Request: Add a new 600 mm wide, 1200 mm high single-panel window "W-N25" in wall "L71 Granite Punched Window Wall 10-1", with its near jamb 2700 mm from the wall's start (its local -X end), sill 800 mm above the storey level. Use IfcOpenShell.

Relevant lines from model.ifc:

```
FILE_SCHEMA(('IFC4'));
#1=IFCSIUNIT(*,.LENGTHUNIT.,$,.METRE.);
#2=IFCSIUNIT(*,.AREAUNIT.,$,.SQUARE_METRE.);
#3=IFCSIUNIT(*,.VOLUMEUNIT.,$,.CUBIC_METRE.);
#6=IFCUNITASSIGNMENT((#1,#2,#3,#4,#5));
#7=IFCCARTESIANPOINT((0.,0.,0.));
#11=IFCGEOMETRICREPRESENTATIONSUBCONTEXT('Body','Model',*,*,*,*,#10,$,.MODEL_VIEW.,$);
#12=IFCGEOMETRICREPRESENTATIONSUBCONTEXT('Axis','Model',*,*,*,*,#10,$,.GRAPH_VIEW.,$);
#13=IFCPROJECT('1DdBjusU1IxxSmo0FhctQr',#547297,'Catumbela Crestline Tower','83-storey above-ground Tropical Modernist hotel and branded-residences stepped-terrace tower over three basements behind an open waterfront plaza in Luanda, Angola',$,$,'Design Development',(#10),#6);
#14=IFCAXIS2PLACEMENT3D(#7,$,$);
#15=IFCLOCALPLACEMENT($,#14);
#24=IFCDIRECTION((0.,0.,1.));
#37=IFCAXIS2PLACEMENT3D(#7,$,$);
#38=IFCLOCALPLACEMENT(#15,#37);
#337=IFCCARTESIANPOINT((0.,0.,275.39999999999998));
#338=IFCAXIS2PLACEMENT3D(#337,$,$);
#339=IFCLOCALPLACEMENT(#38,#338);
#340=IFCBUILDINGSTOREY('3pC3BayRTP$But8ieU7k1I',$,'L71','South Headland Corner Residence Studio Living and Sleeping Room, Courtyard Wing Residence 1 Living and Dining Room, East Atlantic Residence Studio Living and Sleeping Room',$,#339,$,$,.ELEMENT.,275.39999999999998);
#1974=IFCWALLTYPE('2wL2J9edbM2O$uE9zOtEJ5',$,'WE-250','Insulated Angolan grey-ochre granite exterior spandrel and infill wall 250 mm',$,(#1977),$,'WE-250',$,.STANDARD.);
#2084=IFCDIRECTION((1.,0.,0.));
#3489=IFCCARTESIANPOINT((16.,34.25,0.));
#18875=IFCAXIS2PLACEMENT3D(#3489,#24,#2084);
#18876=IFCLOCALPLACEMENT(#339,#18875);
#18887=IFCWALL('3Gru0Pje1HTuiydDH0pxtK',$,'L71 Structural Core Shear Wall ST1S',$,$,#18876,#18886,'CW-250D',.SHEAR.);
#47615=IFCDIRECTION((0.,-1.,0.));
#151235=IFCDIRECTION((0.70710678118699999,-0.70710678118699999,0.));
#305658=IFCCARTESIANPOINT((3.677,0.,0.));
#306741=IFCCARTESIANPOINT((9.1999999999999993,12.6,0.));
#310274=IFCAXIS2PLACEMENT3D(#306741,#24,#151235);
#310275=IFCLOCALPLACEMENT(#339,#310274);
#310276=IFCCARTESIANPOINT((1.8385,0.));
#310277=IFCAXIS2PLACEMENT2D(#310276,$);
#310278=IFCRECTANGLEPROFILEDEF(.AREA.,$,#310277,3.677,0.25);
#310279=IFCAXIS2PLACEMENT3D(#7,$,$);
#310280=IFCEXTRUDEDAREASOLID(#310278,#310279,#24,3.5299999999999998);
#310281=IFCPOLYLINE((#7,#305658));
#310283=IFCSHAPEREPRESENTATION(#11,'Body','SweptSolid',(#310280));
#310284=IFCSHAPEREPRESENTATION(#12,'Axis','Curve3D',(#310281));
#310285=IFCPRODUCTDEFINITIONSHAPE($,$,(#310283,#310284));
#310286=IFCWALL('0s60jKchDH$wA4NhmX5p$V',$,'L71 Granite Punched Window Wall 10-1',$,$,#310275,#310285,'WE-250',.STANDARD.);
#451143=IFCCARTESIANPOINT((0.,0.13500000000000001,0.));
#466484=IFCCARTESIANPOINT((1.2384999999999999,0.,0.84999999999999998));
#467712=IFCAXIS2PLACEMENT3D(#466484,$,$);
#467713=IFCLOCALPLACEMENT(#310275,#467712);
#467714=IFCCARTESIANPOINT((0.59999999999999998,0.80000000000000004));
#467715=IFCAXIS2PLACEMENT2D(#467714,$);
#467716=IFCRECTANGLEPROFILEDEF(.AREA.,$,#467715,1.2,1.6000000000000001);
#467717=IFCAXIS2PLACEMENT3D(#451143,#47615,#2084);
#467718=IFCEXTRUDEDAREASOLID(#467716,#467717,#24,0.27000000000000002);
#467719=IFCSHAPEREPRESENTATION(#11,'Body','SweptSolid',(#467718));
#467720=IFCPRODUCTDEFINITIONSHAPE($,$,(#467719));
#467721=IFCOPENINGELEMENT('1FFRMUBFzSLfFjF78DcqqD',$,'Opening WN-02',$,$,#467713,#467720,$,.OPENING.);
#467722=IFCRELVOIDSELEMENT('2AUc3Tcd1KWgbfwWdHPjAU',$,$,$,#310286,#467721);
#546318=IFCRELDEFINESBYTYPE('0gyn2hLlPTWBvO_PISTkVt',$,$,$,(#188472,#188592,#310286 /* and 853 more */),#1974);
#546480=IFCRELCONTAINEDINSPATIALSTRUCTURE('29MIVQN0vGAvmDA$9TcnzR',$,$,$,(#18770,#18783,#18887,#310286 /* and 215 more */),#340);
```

```python
import numpy as np
import ifcopenshell
import ifcopenshell.api.feature
import ifcopenshell.api.geometry
import ifcopenshell.api.root
import ifcopenshell.api.spatial
import ifcopenshell.geom
import ifcopenshell.util.element
import ifcopenshell.util.placement
import ifcopenshell.util.representation
import ifcopenshell.util.shape
import ifcopenshell.util.unit

model = ifcopenshell.open("model.ifc")
unit_scale = ifcopenshell.util.unit.calculate_unit_scale(model)
settings = ifcopenshell.geom.settings()


def volume(element):
    """Net volume in cubic metres, openings subtracted."""
    shape = ifcopenshell.geom.create_shape(settings, element)
    return ifcopenshell.util.shape.get_volume(shape.geometry)


wall = model.by_guid("0s60jKchDH$wA4NhmX5p$V")
storey = ifcopenshell.util.element.get_container(wall, ifc_class="IfcBuildingStorey")
context = ifcopenshell.util.representation.get_context(model, "Model", "Body", "MODEL_VIEW")
before = volume(wall)

width, height, from_end, sill = 0.6, 1.2, 2.7, 0.8  # metres

# The wall runs along its own X axis, and the end named is its -X end.
wall_shape = ifcopenshell.geom.create_shape(settings, wall)
x, y, z = ifcopenshell.util.shape.get_vertices(wall_shape.geometry).T
start = x.min() + from_end
face, thickness = float(y.min()), float(y.max() - y.min())
wall_matrix = ifcopenshell.util.placement.get_local_placement(wall.ObjectPlacement)
level = ifcopenshell.util.placement.get_local_placement(storey.ObjectPlacement)[2, 3]


def in_wall(x, y):
    """Placement at x, y metres in the wall's axes, at sill height."""
    matrix = wall_matrix.copy()
    matrix[:, 3] = wall_matrix @ np.array([x / unit_scale, y / unit_scale, 0.0, 1.0])
    matrix[2, 3] = level + sill / unit_scale
    return matrix


# Opening: a box that overshoots both wall faces by 50 mm.
opening = ifcopenshell.api.root.create_entity(model, ifc_class="IfcOpeningElement", predefined_type="OPENING")
box = ifcopenshell.api.geometry.add_wall_representation(
    model, context=context, length=width, height=height, thickness=thickness + 0.1
)
ifcopenshell.api.geometry.assign_representation(model, product=opening, representation=box)
ifcopenshell.api.geometry.edit_object_placement(model, product=opening, matrix=in_wall(start, face - 0.05), is_si=False)
ifcopenshell.api.feature.add_feature(model, feature=opening, element=wall)

window = ifcopenshell.api.root.create_entity(model, ifc_class="IfcWindow", name="W-N25", predefined_type="WINDOW")
window.OverallWidth, window.OverallHeight = width / unit_scale, height / unit_scale
window.PartitioningType = "SINGLE_PANEL"
body = ifcopenshell.api.geometry.add_window_representation(
    model,
    context=context,
    overall_width=window.OverallWidth,
    overall_height=window.OverallHeight,
    partition_type="SINGLE_PANEL",
)
ifcopenshell.api.geometry.assign_representation(model, product=window, representation=body)
ifcopenshell.api.spatial.assign_container(model, products=[window], relating_structure=storey)
ifcopenshell.api.feature.add_filling(model, opening=opening, element=window)

# Centre the window in the wall's thickness.
ifcopenshell.api.geometry.edit_object_placement(model, product=window, matrix=in_wall(start, face), is_si=False)
window_shape = ifcopenshell.geom.create_shape(settings, window)
depth = ifcopenshell.util.shape.get_vertices(window_shape.geometry)[:, 1]
offset = face + thickness / 2 - (depth.min() + depth.max()) / 2
ifcopenshell.api.geometry.edit_object_placement(model, product=window, matrix=in_wall(start, offset), is_si=False)

after = volume(wall)

print(f"wall volume {before:.3f} -> {after:.3f} m3")

model.write("model-out.ifc")
```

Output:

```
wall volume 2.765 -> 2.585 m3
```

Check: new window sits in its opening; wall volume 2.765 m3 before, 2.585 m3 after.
